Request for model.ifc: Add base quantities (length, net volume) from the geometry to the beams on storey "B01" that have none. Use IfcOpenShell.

First a look at what the model holds.

```python
import ifcopenshell
import ifcopenshell.util.element
import ifcopenshell.util.unit

model = ifcopenshell.open("model.ifc")
print(model.schema)
for unit_type in ("LENGTHUNIT", "AREAUNIT", "VOLUMEUNIT"):
    print(unit_type, ifcopenshell.util.unit.calculate_unit_scale(model, unit_type))
storey = next(s for s in model.by_type("IfcBuildingStorey") if s.Name == "B01")
beams = [e for e in ifcopenshell.util.element.get_decomposition(storey) if e.is_a("IfcBeam")]
for e in sorted(beams, key=lambda e: e.id()):
    print(e.id(), e.is_a(), e.Name, list(ifcopenshell.util.element.get_psets(e, qtos_only=True)), sep=" | ")
```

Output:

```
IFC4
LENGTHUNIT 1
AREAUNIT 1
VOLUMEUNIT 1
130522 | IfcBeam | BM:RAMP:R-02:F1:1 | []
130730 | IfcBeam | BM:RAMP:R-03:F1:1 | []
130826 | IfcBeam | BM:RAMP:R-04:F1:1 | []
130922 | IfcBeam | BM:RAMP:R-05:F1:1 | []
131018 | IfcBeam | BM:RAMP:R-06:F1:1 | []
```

```python
import ifcopenshell
import ifcopenshell.api.pset
import ifcopenshell.geom
import ifcopenshell.util.element
import ifcopenshell.util.shape
import ifcopenshell.util.unit

model = ifcopenshell.open("model.ifc")
unit_scale = ifcopenshell.util.unit.calculate_unit_scale(model)
volume_scale = ifcopenshell.util.unit.calculate_unit_scale(model, "VOLUMEUNIT")
settings = ifcopenshell.geom.settings()

storey = next(s for s in model.by_type("IfcBuildingStorey") if s.Name == "B01")
beams = [e for e in ifcopenshell.util.element.get_decomposition(storey) if e.is_a("IfcBeam")]

for e in sorted(beams, key=lambda e: e.id()):
    if ifcopenshell.util.element.get_psets(e, qtos_only=True, should_inherit=False):
        continue
    # Geometry comes back in metres, in the element's own axes.
    shape = ifcopenshell.geom.create_shape(settings, e)
    values = {
        "Length": ifcopenshell.util.shape.get_max_xyz(shape.geometry) / unit_scale,
        "NetVolume": ifcopenshell.util.shape.get_volume(shape.geometry) / volume_scale,
    }
    qto = ifcopenshell.api.pset.add_qto(model, product=e, name="Qto_BeamBaseQuantities")
    ifcopenshell.api.pset.edit_qto(model, qto=qto, properties=values)
    print(e.id(), {k: round(v, 3) for k, v in values.items()})

model.write("model_updated.ifc")
```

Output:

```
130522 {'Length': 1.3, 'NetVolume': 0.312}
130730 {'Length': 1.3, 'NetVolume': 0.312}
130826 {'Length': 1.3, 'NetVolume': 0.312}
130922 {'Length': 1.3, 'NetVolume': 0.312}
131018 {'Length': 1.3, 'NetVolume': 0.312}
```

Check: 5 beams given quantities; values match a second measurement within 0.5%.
